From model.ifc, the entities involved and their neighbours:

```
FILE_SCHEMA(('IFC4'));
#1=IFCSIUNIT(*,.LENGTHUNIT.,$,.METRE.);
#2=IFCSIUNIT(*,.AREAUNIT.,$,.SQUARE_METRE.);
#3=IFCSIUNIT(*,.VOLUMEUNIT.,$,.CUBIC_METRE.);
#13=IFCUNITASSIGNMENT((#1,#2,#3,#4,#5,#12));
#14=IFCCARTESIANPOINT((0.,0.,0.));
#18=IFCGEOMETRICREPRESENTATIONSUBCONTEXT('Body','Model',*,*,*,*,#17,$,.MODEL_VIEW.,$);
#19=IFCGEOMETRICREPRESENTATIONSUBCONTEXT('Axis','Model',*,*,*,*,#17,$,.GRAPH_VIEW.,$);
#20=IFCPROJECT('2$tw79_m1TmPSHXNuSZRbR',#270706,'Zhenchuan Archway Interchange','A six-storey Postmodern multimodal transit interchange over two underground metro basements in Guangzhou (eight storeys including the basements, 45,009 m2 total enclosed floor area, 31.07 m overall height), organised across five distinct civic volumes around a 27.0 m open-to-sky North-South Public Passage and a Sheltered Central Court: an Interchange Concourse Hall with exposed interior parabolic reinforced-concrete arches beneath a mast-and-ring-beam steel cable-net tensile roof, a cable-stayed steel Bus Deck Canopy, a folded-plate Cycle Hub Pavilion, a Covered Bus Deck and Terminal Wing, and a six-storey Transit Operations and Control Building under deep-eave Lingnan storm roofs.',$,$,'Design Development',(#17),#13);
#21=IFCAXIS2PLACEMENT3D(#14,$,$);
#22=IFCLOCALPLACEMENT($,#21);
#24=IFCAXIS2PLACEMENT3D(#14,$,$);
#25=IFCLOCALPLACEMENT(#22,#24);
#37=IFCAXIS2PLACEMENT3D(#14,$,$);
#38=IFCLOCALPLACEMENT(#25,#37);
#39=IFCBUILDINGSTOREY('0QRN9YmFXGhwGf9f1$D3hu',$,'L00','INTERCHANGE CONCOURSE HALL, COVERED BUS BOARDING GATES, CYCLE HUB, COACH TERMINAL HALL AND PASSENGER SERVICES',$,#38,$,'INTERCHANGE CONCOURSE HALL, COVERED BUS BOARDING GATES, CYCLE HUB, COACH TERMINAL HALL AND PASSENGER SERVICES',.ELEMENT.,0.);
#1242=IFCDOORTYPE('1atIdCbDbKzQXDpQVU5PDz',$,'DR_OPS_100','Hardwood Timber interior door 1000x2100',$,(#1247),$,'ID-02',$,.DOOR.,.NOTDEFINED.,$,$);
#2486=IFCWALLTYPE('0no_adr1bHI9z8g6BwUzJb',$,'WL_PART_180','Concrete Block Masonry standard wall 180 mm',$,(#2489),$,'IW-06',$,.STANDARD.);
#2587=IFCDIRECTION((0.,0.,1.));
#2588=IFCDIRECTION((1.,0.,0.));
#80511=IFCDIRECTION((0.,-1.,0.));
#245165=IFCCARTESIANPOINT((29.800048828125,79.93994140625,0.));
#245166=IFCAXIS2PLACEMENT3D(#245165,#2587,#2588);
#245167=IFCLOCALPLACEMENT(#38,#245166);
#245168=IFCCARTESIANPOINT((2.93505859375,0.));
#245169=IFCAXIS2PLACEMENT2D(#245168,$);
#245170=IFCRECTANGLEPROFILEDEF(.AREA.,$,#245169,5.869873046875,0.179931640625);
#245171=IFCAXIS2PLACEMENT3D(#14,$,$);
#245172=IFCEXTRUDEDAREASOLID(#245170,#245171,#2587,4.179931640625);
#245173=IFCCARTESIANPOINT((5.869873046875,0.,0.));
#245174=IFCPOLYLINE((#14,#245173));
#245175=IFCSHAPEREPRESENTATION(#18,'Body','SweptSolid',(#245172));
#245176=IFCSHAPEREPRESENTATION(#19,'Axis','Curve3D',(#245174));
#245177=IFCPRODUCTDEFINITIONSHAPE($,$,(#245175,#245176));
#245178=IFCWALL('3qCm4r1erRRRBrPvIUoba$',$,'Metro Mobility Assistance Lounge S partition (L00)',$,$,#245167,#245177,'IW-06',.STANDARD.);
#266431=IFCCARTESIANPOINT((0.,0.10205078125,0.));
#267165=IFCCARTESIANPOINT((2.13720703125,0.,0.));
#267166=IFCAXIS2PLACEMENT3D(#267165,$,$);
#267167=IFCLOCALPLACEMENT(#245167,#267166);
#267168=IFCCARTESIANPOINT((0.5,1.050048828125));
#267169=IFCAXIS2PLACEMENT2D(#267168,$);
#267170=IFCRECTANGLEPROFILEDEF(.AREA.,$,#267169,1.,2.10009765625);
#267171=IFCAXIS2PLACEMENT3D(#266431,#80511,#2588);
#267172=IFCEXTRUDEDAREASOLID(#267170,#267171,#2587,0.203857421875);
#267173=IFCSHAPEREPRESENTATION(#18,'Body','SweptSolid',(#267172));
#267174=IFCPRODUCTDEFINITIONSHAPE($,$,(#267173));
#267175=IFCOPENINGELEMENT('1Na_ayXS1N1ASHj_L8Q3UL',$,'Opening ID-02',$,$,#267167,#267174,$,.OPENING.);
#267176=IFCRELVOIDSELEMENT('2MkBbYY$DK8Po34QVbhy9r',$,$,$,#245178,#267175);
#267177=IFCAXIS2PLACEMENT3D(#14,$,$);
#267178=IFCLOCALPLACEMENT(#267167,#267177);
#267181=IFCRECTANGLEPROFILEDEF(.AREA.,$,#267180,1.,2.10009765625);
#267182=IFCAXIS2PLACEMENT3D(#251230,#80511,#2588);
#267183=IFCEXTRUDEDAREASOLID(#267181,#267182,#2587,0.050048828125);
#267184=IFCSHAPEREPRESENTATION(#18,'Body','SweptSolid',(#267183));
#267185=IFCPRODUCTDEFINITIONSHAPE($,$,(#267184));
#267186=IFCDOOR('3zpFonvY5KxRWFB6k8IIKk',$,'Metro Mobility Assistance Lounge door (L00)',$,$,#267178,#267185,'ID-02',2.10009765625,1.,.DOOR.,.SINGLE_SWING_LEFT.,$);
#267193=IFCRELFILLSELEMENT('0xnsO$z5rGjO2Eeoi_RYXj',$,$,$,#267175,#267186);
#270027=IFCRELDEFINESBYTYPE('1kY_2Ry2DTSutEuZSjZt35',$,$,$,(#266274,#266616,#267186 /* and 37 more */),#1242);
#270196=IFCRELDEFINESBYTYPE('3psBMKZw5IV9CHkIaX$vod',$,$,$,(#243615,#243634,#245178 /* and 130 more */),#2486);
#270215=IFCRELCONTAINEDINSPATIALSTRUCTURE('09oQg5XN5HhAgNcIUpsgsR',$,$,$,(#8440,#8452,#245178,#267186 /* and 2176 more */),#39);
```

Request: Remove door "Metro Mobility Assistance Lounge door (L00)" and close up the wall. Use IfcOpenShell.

```python
import ifcopenshell
import ifcopenshell.api.feature
import ifcopenshell.api.root
import ifcopenshell.geom
import ifcopenshell.util.shape

model = ifcopenshell.open("model.ifc")
settings = ifcopenshell.geom.settings()


def volume(element):
    """Net volume in cubic metres, openings subtracted."""
    shape = ifcopenshell.geom.create_shape(settings, element)
    return ifcopenshell.util.shape.get_volume(shape.geometry)


door = model.by_guid("3zpFonvY5KxRWFB6k8IIKk")
opening = door.FillsVoids[0].RelatingOpeningElement
wall = opening.VoidsElements[0].RelatingBuildingElement
before = volume(wall)

ifcopenshell.api.root.remove_product(model, product=door)
ifcopenshell.api.feature.remove_feature(model, feature=opening)

after = volume(wall)

print(f"wall volume {before:.3f} -> {after:.3f} m3")

model.write("model_rev.ifc")
```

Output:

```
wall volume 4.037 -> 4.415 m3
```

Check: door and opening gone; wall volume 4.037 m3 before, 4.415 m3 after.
